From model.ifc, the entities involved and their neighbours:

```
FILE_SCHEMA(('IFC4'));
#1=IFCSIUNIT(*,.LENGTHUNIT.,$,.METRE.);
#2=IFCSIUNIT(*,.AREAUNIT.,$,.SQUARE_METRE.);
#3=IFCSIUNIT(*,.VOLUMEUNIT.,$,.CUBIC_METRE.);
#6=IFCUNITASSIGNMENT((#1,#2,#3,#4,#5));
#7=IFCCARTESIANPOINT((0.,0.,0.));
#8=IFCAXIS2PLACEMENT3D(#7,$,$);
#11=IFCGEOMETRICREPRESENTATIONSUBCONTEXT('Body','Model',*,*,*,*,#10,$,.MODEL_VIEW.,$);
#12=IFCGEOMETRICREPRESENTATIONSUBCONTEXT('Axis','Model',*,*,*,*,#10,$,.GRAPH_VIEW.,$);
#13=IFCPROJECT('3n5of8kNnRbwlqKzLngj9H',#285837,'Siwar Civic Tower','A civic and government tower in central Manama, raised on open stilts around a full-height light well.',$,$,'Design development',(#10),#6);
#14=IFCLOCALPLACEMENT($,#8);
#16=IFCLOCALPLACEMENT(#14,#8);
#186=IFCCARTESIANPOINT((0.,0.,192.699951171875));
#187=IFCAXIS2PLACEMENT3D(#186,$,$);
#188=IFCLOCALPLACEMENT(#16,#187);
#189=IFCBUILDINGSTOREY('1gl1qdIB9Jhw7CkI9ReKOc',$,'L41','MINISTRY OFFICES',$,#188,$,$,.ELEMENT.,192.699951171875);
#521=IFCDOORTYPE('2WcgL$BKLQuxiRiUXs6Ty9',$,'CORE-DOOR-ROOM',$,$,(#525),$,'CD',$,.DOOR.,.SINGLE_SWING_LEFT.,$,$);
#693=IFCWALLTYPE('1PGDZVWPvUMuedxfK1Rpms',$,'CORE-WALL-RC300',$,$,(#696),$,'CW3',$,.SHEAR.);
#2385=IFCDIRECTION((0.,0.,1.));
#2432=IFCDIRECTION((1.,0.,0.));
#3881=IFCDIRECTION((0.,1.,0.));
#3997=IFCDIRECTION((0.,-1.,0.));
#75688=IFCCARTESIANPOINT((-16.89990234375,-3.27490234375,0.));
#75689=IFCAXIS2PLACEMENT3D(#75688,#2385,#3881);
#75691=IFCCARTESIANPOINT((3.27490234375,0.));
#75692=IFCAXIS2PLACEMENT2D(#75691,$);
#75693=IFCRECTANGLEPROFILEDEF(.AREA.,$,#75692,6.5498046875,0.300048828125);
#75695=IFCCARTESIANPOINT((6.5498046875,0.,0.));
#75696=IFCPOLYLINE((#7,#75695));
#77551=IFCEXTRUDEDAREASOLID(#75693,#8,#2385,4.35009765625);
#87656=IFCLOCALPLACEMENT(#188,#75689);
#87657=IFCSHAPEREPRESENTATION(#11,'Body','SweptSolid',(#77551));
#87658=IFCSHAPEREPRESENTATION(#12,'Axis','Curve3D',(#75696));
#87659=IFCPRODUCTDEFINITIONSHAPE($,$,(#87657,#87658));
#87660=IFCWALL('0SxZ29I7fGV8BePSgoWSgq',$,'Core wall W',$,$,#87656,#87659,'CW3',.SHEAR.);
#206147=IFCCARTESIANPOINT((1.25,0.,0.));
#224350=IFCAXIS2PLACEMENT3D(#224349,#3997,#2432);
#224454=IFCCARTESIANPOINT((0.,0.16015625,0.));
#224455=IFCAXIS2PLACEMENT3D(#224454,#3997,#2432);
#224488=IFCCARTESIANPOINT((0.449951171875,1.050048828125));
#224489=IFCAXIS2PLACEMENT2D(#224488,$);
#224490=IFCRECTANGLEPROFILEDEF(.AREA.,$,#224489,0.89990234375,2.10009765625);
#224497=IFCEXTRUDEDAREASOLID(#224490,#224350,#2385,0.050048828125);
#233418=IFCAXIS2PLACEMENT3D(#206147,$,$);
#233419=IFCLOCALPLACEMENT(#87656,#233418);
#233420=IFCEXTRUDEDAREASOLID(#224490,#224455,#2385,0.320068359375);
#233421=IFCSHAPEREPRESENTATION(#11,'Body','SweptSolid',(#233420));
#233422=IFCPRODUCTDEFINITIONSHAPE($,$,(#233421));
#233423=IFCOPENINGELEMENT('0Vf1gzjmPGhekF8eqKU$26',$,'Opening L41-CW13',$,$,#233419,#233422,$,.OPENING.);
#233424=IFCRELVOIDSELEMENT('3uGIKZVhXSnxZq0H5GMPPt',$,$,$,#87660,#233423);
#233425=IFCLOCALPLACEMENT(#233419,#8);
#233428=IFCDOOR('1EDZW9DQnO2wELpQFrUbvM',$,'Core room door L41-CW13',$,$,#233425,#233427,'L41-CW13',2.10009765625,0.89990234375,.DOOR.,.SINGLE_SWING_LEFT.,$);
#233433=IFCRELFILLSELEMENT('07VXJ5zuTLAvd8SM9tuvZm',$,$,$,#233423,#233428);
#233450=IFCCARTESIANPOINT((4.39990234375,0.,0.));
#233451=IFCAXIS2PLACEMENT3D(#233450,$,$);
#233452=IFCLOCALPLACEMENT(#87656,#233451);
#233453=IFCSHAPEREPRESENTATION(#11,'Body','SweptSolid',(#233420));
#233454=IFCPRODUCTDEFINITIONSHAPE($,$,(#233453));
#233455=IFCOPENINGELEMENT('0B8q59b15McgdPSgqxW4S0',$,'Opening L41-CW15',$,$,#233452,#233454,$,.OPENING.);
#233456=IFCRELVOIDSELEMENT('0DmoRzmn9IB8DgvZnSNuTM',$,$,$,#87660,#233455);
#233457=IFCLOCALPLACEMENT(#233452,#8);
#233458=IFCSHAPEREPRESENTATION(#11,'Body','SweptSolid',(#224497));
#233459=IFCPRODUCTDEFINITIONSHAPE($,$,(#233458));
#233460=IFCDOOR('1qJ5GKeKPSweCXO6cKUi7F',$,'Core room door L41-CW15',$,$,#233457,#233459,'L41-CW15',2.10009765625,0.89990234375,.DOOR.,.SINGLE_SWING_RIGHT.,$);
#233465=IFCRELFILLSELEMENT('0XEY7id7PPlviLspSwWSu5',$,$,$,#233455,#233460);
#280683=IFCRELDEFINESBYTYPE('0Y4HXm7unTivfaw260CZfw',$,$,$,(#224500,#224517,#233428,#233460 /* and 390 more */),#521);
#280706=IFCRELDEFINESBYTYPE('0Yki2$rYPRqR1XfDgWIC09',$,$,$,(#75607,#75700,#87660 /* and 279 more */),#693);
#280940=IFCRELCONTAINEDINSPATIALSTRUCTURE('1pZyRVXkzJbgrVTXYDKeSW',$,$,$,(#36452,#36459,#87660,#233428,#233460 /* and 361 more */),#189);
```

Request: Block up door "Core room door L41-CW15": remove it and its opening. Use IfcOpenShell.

```python
import ifcopenshell
import ifcopenshell.api.feature
import ifcopenshell.api.root
import ifcopenshell.geom
import ifcopenshell.util.shape

model = ifcopenshell.open("model.ifc")
settings = ifcopenshell.geom.settings()


def volume(element):
    """Net volume in cubic metres, openings subtracted."""
    shape = ifcopenshell.geom.create_shape(settings, element)
    return ifcopenshell.util.shape.get_volume(shape.geometry)


door = model.by_guid("1qJ5GKeKPSweCXO6cKUi7F")
opening = door.FillsVoids[0].RelatingOpeningElement
wall = opening.VoidsElements[0].RelatingBuildingElement
before = volume(wall)

ifcopenshell.api.root.remove_product(model, product=door)
ifcopenshell.api.feature.remove_feature(model, feature=opening)

after = volume(wall)

print(f"wall volume {before:.3f} -> {after:.3f} m3")

model.write("model_edited.ifc")
```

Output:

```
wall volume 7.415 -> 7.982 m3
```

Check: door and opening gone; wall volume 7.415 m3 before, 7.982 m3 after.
